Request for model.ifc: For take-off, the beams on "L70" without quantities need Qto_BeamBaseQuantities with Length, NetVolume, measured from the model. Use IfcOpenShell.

First a look at what the model holds.

```python
import ifcopenshell
import ifcopenshell.util.element
import ifcopenshell.util.unit

model = ifcopenshell.open("model.ifc")
print(model.schema)
for unit_type in ("LENGTHUNIT", "AREAUNIT", "VOLUMEUNIT"):
    print(unit_type, ifcopenshell.util.unit.calculate_unit_scale(model, unit_type))
storey = next(s for s in model.by_type("IfcBuildingStorey") if s.Name == "L70")
beams = [e for e in ifcopenshell.util.element.get_decomposition(storey) if e.is_a("IfcBeam")]
for e in sorted(beams, key=lambda e: e.id()):
    print(e.id(), e.is_a(), e.Name, list(ifcopenshell.util.element.get_psets(e, qtos_only=True)), sep=" | ")
```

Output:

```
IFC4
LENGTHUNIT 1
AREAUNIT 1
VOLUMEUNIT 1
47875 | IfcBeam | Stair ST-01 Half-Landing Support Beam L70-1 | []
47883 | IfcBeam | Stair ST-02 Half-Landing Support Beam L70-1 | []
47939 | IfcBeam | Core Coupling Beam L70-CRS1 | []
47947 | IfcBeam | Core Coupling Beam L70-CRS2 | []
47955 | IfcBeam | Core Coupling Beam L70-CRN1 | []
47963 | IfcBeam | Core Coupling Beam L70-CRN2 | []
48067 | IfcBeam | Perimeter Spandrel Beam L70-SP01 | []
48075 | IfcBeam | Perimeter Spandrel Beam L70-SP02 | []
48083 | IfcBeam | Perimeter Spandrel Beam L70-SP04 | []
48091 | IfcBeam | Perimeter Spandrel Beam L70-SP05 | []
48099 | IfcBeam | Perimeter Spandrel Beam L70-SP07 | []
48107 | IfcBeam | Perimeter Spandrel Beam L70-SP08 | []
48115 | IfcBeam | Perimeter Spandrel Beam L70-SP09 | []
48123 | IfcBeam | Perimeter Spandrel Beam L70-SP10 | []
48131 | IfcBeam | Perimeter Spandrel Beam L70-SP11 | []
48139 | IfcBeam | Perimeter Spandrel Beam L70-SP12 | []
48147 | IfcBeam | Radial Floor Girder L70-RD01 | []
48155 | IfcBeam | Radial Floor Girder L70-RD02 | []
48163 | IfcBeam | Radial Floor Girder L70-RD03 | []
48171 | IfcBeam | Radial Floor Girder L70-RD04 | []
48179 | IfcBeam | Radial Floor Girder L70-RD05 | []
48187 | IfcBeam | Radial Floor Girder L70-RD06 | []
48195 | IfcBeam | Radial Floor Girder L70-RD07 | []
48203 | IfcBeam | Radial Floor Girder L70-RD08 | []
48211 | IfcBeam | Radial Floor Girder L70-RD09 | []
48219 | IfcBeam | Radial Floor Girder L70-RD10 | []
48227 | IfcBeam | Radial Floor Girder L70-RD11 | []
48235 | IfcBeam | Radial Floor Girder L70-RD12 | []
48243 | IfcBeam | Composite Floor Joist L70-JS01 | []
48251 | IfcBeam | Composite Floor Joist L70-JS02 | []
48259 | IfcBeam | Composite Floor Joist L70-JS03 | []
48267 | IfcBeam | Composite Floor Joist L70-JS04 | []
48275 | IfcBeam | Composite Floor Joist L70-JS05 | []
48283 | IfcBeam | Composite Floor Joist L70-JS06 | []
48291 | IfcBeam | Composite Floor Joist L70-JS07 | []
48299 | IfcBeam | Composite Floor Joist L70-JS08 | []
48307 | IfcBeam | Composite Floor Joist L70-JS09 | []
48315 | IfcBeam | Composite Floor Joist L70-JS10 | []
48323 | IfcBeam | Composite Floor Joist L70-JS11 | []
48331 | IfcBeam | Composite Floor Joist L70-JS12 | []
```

```python
import ifcopenshell
import ifcopenshell.api.pset
import ifcopenshell.geom
import ifcopenshell.util.element
import ifcopenshell.util.shape
import ifcopenshell.util.unit

model = ifcopenshell.open("model.ifc")
unit_scale = ifcopenshell.util.unit.calculate_unit_scale(model)
volume_scale = ifcopenshell.util.unit.calculate_unit_scale(model, "VOLUMEUNIT")
settings = ifcopenshell.geom.settings()

storey = next(s for s in model.by_type("IfcBuildingStorey") if s.Name == "L70")
beams = [e for e in ifcopenshell.util.element.get_decomposition(storey) if e.is_a("IfcBeam")]

for e in sorted(beams, key=lambda e: e.id()):
    if ifcopenshell.util.element.get_psets(e, qtos_only=True, should_inherit=False):
        continue
    # Geometry comes back in metres, in the element's own axes.
    shape = ifcopenshell.geom.create_shape(settings, e)
    values = {
        "Length": ifcopenshell.util.shape.get_max_xyz(shape.geometry) / unit_scale,
        "NetVolume": ifcopenshell.util.shape.get_volume(shape.geometry) / volume_scale,
    }
    qto = ifcopenshell.api.pset.add_qto(model, product=e, name="Qto_BeamBaseQuantities")
    ifcopenshell.api.pset.edit_qto(model, qto=qto, properties=values)
    print(e.id(), {k: round(v, 3) for k, v in values.items()})

model.write("model_v2.ifc")
```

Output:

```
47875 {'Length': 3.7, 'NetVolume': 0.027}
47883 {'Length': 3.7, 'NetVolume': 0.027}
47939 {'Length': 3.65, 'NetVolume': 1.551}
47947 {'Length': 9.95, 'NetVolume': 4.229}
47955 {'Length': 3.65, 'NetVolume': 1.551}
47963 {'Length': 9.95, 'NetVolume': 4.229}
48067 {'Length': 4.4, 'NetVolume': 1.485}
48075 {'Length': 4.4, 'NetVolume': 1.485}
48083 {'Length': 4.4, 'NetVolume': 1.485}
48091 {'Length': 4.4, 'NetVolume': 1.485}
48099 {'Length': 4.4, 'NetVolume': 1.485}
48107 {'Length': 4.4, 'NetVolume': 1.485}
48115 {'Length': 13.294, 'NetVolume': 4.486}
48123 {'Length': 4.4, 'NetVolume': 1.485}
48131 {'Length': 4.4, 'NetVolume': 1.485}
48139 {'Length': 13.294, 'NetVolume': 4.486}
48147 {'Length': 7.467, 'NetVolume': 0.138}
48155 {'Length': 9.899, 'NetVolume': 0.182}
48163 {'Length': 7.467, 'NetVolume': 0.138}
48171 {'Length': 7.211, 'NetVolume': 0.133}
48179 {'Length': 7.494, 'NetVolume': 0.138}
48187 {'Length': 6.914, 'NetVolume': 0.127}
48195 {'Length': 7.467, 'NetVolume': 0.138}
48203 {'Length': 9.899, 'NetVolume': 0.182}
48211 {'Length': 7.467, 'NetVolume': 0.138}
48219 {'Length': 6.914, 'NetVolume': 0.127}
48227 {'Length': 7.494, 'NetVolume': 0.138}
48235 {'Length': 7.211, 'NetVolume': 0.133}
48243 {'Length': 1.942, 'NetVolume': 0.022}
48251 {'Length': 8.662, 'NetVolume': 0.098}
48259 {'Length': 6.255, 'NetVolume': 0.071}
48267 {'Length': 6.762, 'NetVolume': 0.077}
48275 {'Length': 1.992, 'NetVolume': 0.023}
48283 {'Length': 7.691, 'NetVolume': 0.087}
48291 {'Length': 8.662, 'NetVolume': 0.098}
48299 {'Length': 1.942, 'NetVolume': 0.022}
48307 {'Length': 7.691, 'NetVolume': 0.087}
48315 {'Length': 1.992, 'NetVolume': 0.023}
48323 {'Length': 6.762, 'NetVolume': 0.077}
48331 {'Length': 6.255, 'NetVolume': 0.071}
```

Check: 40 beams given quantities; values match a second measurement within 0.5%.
